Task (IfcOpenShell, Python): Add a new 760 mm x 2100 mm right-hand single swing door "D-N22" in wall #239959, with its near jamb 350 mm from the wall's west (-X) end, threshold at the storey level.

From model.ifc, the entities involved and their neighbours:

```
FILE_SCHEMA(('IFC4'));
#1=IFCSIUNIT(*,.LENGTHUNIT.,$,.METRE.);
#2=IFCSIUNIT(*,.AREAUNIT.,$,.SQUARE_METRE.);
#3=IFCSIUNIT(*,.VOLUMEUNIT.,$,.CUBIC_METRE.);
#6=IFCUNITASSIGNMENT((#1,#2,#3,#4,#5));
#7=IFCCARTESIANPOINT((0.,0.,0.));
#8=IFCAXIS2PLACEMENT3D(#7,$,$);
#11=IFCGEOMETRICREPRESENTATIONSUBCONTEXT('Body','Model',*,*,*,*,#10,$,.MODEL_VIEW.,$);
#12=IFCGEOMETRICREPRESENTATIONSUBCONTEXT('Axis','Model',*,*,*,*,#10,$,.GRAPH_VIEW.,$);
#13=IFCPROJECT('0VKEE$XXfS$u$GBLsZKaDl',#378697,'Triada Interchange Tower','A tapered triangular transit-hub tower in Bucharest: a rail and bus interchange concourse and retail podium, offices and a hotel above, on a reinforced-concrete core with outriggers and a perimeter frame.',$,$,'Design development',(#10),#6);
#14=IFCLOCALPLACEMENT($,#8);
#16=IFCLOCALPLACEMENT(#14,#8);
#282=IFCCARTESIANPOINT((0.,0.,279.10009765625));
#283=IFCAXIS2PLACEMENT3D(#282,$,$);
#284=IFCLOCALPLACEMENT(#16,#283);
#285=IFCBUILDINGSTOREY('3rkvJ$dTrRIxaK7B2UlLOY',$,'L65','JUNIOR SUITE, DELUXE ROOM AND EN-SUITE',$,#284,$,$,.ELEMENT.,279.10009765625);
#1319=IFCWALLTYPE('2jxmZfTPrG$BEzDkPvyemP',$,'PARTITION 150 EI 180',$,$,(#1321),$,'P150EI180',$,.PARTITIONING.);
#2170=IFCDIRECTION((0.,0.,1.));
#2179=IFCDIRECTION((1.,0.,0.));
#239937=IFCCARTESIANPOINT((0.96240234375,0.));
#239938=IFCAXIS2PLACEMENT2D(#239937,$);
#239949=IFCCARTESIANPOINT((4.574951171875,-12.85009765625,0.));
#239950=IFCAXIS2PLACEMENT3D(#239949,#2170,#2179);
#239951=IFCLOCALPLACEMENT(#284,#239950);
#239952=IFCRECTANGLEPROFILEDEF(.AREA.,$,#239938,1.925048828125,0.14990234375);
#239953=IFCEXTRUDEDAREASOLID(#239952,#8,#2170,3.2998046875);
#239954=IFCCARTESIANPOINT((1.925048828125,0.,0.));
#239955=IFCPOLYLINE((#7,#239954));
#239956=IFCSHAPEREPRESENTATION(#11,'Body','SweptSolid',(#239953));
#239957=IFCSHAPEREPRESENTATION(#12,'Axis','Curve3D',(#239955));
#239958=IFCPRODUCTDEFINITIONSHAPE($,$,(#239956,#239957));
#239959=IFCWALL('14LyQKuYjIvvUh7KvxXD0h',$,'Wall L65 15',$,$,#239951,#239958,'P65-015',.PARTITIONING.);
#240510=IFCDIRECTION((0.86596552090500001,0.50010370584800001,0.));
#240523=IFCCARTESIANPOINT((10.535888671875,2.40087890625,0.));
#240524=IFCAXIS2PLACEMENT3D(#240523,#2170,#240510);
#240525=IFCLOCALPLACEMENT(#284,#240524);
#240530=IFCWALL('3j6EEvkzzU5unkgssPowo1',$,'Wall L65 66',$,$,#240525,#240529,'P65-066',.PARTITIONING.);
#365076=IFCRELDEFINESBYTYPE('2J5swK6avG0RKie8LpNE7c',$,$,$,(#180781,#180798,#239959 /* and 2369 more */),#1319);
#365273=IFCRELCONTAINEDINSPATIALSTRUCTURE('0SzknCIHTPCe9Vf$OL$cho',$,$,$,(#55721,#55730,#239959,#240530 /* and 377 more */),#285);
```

```python
import numpy as np
import ifcopenshell
import ifcopenshell.api.feature
import ifcopenshell.api.geometry
import ifcopenshell.api.root
import ifcopenshell.api.spatial
import ifcopenshell.geom
import ifcopenshell.util.element
import ifcopenshell.util.placement
import ifcopenshell.util.representation
import ifcopenshell.util.shape
import ifcopenshell.util.unit

model = ifcopenshell.open("model.ifc")
unit_scale = ifcopenshell.util.unit.calculate_unit_scale(model)
settings = ifcopenshell.geom.settings()


def volume(element):
    """Net volume in cubic metres, openings subtracted."""
    shape = ifcopenshell.geom.create_shape(settings, element)
    return ifcopenshell.util.shape.get_volume(shape.geometry)


wall = model.by_id(239959)
storey = ifcopenshell.util.element.get_container(wall, ifc_class="IfcBuildingStorey")
context = ifcopenshell.util.representation.get_context(model, "Model", "Body", "MODEL_VIEW")
before = volume(wall)

width, height, from_end, sill = 0.76, 2.1, 0.35, 0.0  # metres

# The wall runs along its own X axis, and the end named is its -X end.
wall_shape = ifcopenshell.geom.create_shape(settings, wall)
x, y, z = ifcopenshell.util.shape.get_vertices(wall_shape.geometry).T
start = x.min() + from_end
face, thickness = float(y.min()), float(y.max() - y.min())
wall_matrix = ifcopenshell.util.placement.get_local_placement(wall.ObjectPlacement)
level = ifcopenshell.util.placement.get_local_placement(storey.ObjectPlacement)[2, 3]


def in_wall(x, y):
    """Placement at x, y metres in the wall's axes, at sill height."""
    matrix = wall_matrix.copy()
    matrix[:, 3] = wall_matrix @ np.array([x / unit_scale, y / unit_scale, 0.0, 1.0])
    matrix[2, 3] = level + sill / unit_scale
    return matrix


# Opening: a box that overshoots both wall faces by 50 mm.
opening = ifcopenshell.api.root.create_entity(model, ifc_class="IfcOpeningElement", predefined_type="OPENING")
box = ifcopenshell.api.geometry.add_wall_representation(
    model, context=context, length=width, height=height, thickness=thickness + 0.1
)
ifcopenshell.api.geometry.assign_representation(model, product=opening, representation=box)
ifcopenshell.api.geometry.edit_object_placement(model, product=opening, matrix=in_wall(start, face - 0.05), is_si=False)
ifcopenshell.api.feature.add_feature(model, feature=opening, element=wall)

door = ifcopenshell.api.root.create_entity(model, ifc_class="IfcDoor", name="D-N22", predefined_type="DOOR")
door.OverallWidth, door.OverallHeight = width / unit_scale, height / unit_scale
door.OperationType = "SINGLE_SWING_RIGHT"
body = ifcopenshell.api.geometry.add_door_representation(
    model,
    context=context,
    overall_width=door.OverallWidth,
    overall_height=door.OverallHeight,
    operation_type="SINGLE_SWING_RIGHT",
    lining_properties={"LiningDepth": thickness / unit_scale, "ThresholdDepth": thickness / unit_scale},
)
ifcopenshell.api.geometry.assign_representation(model, product=door, representation=body)
ifcopenshell.api.spatial.assign_container(model, products=[door], relating_structure=storey)
ifcopenshell.api.feature.add_filling(model, opening=opening, element=door)

# The lining spans the wall, so the door starts at the wall face.
ifcopenshell.api.geometry.edit_object_placement(model, product=door, matrix=in_wall(start, face), is_si=False)

after = volume(wall)

print(f"wall volume {before:.3f} -> {after:.3f} m3")

model.write("model_edited.ifc")
```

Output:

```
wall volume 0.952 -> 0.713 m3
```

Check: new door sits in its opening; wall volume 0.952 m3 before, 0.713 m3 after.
